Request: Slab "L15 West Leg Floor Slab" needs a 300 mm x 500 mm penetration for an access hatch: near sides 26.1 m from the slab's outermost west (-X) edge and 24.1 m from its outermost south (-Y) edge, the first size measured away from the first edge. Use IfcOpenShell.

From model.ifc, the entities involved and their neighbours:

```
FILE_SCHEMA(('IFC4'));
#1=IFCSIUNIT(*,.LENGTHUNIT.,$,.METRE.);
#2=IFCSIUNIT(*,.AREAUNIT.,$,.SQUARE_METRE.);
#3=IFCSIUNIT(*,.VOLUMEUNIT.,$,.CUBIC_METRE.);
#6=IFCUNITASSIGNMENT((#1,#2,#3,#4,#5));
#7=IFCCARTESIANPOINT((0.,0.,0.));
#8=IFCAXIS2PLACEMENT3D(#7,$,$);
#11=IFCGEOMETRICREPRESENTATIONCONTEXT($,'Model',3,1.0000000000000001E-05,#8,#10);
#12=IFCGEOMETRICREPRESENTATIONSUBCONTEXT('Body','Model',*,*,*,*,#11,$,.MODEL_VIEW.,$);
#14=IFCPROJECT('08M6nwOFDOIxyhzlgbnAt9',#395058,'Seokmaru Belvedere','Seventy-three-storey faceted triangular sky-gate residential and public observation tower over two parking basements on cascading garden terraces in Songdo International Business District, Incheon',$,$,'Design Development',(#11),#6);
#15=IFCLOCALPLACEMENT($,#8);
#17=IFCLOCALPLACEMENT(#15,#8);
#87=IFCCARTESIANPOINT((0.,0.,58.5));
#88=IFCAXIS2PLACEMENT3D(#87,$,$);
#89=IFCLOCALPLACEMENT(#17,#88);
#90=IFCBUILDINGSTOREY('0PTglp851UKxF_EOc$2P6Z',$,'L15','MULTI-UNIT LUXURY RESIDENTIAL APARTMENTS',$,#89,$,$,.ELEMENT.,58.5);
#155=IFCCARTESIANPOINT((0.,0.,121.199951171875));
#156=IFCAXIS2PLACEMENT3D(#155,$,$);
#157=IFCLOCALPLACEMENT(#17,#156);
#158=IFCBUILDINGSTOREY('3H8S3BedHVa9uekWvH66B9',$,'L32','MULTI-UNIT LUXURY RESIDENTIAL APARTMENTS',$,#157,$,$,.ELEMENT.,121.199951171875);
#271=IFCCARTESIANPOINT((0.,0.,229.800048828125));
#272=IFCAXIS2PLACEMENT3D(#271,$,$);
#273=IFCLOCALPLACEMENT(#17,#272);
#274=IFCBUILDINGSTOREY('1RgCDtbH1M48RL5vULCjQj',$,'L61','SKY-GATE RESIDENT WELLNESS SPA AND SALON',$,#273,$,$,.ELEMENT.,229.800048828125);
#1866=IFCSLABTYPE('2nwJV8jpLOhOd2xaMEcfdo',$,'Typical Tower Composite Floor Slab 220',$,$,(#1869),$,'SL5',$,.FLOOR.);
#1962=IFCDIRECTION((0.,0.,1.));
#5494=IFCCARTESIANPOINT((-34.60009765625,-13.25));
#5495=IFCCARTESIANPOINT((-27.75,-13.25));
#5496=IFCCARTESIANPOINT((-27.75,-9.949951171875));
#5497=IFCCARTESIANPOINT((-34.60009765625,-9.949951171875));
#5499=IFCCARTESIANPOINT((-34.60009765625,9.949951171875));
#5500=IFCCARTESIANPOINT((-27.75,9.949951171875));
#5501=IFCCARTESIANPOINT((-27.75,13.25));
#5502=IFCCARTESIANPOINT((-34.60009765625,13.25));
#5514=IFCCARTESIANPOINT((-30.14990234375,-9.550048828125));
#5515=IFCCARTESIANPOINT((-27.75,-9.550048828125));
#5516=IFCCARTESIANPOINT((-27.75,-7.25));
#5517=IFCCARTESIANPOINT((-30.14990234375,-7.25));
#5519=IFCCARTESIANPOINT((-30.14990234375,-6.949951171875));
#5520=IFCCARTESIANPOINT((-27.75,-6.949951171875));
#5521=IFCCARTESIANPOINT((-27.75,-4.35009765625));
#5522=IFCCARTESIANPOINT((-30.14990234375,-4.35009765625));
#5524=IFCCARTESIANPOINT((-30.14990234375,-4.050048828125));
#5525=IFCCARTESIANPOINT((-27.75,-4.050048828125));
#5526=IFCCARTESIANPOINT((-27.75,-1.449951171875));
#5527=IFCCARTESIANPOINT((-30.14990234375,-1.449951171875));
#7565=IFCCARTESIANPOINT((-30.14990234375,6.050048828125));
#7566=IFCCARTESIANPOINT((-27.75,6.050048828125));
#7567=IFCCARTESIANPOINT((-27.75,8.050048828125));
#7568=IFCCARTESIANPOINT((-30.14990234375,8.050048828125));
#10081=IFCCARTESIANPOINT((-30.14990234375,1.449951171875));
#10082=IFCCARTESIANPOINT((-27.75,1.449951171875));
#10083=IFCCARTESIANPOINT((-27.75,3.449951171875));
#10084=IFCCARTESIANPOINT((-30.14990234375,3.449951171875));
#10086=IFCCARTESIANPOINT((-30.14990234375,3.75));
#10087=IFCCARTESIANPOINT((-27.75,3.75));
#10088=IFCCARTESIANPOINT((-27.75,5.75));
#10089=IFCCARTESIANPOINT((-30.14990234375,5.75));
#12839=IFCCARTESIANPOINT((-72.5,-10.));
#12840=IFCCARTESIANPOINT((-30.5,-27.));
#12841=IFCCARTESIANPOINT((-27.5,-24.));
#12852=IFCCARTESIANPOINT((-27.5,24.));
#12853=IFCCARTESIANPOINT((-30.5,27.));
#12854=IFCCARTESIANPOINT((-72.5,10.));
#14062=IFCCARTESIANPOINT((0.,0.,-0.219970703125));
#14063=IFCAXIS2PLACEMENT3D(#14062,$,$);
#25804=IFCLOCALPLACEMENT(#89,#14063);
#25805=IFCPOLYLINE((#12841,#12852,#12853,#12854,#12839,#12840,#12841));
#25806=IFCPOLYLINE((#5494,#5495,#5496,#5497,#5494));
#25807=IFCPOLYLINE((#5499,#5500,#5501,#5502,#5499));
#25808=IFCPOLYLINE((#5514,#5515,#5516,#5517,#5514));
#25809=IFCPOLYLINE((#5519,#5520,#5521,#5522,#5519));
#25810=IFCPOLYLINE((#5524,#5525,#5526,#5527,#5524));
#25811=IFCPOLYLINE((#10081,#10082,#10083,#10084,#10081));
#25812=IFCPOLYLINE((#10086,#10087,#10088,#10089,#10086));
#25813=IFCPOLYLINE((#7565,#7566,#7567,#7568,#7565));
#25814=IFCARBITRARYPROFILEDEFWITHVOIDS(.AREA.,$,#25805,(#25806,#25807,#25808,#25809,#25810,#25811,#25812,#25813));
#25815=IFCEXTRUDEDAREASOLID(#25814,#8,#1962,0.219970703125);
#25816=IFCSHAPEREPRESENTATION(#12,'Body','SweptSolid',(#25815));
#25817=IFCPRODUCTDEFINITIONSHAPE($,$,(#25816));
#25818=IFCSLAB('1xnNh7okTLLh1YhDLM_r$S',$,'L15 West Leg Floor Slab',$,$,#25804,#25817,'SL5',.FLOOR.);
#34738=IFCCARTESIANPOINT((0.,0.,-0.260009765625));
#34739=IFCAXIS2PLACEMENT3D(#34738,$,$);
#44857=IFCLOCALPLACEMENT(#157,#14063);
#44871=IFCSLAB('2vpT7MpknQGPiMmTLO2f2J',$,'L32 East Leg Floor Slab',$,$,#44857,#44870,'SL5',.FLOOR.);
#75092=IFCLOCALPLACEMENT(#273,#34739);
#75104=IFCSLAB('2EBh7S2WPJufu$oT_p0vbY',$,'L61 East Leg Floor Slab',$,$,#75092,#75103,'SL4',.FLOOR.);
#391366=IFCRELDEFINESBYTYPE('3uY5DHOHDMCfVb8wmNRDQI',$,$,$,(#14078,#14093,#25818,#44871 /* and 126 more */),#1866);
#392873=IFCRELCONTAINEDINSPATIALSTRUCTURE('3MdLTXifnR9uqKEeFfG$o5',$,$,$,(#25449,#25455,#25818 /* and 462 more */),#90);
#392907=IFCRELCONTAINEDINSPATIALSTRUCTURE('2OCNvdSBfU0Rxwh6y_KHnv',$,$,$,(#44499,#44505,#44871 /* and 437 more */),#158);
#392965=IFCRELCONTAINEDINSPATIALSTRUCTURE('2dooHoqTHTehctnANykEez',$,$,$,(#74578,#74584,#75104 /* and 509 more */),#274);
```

```python
import numpy as np
import ifcopenshell
import ifcopenshell.api.feature
import ifcopenshell.api.geometry
import ifcopenshell.api.root
import ifcopenshell.geom
import ifcopenshell.util.placement
import ifcopenshell.util.representation
import ifcopenshell.util.shape
import ifcopenshell.util.unit

model = ifcopenshell.open("model.ifc")
unit_scale = ifcopenshell.util.unit.calculate_unit_scale(model)
settings = ifcopenshell.geom.settings()


def volume(element):
    """Net volume in cubic metres, openings subtracted."""
    shape = ifcopenshell.geom.create_shape(settings, element)
    return ifcopenshell.util.shape.get_volume(shape.geometry)


slab = model.by_guid("1xnNh7okTLLh1YhDLM_r$S")
before = volume(slab)

# Extent in the slab's own axes, in metres. The edges named are its -X and -Y sides.
slab_shape = ifcopenshell.geom.create_shape(settings, slab)
vertices = ifcopenshell.util.shape.get_vertices(slab_shape.geometry)
x_min, y_min, bottom = vertices.min(axis=0)
top = vertices[:, 2].max()

opening = ifcopenshell.api.root.create_entity(model, ifc_class="IfcOpeningElement", name="Access hatch opening", predefined_type="OPENING")
context = ifcopenshell.util.representation.get_context(model, "Model", "Body", "MODEL_VIEW")
width, depth = 0.3, 0.5
outline = [(0.0, 0.0), (width, 0.0), (width, depth), (0.0, depth), (0.0, 0.0)]
# Overshoot both faces by 50 mm so the cut is clean.
shape = ifcopenshell.api.geometry.add_slab_representation(
    model, context=context, depth=top - bottom + 0.1, polyline=outline
)
ifcopenshell.api.geometry.assign_representation(model, product=opening, representation=shape)

matrix = ifcopenshell.util.placement.get_local_placement(slab.ObjectPlacement)
matrix[:, 3] = matrix @ np.append(np.array([x_min + 26.1, y_min + 24.1, bottom - 0.05]) / unit_scale, 1.0)
ifcopenshell.api.geometry.edit_object_placement(model, product=opening, matrix=matrix, is_si=False)
ifcopenshell.api.feature.add_feature(model, feature=opening, element=slab)

after = volume(slab)

print(f"slab volume {before:.3f} -> {after:.3f} m3")

model.write("model_v2.ifc")
```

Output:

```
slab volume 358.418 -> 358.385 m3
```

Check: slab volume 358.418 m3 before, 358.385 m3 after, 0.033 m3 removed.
